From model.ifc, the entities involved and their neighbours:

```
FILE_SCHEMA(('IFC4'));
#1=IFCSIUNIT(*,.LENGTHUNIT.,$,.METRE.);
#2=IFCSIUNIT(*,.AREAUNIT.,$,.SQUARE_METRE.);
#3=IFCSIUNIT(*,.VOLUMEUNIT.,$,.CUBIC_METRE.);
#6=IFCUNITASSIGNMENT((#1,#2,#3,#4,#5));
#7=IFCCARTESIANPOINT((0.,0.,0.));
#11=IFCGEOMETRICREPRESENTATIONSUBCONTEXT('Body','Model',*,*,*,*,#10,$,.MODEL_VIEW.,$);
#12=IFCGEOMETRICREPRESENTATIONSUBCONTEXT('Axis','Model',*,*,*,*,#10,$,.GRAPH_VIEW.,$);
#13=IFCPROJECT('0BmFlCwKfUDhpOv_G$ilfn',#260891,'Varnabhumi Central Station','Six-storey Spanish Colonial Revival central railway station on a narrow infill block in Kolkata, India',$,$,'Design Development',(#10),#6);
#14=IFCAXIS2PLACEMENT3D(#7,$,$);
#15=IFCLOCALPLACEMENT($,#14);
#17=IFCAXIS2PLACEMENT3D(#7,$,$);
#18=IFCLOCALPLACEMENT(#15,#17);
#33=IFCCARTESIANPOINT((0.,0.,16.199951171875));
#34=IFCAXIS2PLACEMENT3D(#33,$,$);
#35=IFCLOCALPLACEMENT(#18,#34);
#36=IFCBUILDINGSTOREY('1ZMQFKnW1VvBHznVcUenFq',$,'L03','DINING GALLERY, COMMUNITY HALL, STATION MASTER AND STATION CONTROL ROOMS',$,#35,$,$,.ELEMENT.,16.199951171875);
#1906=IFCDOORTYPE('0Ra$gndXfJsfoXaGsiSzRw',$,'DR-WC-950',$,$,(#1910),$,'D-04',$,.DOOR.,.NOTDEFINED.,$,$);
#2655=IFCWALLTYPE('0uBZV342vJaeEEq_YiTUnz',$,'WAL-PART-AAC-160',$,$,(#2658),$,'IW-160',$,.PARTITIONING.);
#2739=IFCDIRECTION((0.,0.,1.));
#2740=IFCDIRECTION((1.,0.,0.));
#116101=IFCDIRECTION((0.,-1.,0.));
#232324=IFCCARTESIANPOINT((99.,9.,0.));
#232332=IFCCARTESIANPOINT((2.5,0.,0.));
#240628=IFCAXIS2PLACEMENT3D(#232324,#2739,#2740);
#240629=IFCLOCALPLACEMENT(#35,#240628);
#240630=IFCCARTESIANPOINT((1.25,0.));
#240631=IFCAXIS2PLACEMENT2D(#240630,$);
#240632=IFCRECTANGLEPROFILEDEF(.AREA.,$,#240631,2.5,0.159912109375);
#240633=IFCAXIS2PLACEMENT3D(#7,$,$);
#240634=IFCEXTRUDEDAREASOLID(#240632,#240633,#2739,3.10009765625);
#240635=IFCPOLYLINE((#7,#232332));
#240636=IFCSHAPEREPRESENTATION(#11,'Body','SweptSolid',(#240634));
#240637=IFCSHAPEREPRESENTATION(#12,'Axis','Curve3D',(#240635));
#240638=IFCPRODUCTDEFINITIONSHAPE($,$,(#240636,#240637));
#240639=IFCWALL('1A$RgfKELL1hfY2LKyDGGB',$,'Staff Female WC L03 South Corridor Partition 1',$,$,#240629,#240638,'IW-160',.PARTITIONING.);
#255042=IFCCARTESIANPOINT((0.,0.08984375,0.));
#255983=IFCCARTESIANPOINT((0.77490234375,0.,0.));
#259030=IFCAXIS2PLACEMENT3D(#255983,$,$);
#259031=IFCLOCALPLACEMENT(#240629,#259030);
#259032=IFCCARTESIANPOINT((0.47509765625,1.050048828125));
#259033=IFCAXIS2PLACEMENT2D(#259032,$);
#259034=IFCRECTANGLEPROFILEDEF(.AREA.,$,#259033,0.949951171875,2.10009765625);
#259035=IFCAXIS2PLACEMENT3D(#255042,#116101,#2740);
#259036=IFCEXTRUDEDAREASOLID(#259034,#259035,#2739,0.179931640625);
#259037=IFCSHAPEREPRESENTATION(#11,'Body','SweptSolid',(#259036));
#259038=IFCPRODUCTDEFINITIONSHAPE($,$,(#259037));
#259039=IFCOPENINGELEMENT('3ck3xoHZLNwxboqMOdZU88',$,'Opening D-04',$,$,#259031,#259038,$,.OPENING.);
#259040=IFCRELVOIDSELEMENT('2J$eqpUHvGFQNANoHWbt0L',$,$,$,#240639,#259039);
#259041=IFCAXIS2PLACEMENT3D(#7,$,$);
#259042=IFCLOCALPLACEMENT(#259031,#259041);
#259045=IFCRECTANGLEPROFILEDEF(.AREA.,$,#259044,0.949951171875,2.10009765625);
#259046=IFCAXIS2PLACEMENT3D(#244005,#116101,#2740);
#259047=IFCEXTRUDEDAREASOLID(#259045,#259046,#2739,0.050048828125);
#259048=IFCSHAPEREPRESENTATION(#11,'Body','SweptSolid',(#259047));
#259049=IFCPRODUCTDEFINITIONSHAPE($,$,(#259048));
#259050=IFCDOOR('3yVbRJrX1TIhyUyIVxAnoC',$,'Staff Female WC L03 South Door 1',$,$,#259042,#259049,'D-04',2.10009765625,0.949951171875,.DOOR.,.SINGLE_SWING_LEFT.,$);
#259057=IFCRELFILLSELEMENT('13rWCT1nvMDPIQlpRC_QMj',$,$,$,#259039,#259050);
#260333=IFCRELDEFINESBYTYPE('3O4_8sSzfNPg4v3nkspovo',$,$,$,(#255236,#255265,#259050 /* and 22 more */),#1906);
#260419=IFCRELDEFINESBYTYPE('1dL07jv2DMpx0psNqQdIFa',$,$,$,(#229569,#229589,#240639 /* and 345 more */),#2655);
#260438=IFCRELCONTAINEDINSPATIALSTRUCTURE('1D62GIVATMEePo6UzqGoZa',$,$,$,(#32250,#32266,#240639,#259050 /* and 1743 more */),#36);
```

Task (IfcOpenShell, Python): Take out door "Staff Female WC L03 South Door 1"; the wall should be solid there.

```python
import ifcopenshell
import ifcopenshell.api.feature
import ifcopenshell.api.root
import ifcopenshell.geom
import ifcopenshell.util.shape

model = ifcopenshell.open("model.ifc")
settings = ifcopenshell.geom.settings()


def volume(element):
    """Net volume in cubic metres, openings subtracted."""
    shape = ifcopenshell.geom.create_shape(settings, element)
    return ifcopenshell.util.shape.get_volume(shape.geometry)


door = model.by_guid("3yVbRJrX1TIhyUyIVxAnoC")
opening = door.FillsVoids[0].RelatingOpeningElement
wall = opening.VoidsElements[0].RelatingBuildingElement
before = volume(wall)

ifcopenshell.api.root.remove_product(model, product=door)
ifcopenshell.api.feature.remove_feature(model, feature=opening)

after = volume(wall)

print(f"wall volume {before:.3f} -> {after:.3f} m3")

model.write("model_v2.ifc")
```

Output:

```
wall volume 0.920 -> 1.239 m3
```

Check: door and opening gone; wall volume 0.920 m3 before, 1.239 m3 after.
